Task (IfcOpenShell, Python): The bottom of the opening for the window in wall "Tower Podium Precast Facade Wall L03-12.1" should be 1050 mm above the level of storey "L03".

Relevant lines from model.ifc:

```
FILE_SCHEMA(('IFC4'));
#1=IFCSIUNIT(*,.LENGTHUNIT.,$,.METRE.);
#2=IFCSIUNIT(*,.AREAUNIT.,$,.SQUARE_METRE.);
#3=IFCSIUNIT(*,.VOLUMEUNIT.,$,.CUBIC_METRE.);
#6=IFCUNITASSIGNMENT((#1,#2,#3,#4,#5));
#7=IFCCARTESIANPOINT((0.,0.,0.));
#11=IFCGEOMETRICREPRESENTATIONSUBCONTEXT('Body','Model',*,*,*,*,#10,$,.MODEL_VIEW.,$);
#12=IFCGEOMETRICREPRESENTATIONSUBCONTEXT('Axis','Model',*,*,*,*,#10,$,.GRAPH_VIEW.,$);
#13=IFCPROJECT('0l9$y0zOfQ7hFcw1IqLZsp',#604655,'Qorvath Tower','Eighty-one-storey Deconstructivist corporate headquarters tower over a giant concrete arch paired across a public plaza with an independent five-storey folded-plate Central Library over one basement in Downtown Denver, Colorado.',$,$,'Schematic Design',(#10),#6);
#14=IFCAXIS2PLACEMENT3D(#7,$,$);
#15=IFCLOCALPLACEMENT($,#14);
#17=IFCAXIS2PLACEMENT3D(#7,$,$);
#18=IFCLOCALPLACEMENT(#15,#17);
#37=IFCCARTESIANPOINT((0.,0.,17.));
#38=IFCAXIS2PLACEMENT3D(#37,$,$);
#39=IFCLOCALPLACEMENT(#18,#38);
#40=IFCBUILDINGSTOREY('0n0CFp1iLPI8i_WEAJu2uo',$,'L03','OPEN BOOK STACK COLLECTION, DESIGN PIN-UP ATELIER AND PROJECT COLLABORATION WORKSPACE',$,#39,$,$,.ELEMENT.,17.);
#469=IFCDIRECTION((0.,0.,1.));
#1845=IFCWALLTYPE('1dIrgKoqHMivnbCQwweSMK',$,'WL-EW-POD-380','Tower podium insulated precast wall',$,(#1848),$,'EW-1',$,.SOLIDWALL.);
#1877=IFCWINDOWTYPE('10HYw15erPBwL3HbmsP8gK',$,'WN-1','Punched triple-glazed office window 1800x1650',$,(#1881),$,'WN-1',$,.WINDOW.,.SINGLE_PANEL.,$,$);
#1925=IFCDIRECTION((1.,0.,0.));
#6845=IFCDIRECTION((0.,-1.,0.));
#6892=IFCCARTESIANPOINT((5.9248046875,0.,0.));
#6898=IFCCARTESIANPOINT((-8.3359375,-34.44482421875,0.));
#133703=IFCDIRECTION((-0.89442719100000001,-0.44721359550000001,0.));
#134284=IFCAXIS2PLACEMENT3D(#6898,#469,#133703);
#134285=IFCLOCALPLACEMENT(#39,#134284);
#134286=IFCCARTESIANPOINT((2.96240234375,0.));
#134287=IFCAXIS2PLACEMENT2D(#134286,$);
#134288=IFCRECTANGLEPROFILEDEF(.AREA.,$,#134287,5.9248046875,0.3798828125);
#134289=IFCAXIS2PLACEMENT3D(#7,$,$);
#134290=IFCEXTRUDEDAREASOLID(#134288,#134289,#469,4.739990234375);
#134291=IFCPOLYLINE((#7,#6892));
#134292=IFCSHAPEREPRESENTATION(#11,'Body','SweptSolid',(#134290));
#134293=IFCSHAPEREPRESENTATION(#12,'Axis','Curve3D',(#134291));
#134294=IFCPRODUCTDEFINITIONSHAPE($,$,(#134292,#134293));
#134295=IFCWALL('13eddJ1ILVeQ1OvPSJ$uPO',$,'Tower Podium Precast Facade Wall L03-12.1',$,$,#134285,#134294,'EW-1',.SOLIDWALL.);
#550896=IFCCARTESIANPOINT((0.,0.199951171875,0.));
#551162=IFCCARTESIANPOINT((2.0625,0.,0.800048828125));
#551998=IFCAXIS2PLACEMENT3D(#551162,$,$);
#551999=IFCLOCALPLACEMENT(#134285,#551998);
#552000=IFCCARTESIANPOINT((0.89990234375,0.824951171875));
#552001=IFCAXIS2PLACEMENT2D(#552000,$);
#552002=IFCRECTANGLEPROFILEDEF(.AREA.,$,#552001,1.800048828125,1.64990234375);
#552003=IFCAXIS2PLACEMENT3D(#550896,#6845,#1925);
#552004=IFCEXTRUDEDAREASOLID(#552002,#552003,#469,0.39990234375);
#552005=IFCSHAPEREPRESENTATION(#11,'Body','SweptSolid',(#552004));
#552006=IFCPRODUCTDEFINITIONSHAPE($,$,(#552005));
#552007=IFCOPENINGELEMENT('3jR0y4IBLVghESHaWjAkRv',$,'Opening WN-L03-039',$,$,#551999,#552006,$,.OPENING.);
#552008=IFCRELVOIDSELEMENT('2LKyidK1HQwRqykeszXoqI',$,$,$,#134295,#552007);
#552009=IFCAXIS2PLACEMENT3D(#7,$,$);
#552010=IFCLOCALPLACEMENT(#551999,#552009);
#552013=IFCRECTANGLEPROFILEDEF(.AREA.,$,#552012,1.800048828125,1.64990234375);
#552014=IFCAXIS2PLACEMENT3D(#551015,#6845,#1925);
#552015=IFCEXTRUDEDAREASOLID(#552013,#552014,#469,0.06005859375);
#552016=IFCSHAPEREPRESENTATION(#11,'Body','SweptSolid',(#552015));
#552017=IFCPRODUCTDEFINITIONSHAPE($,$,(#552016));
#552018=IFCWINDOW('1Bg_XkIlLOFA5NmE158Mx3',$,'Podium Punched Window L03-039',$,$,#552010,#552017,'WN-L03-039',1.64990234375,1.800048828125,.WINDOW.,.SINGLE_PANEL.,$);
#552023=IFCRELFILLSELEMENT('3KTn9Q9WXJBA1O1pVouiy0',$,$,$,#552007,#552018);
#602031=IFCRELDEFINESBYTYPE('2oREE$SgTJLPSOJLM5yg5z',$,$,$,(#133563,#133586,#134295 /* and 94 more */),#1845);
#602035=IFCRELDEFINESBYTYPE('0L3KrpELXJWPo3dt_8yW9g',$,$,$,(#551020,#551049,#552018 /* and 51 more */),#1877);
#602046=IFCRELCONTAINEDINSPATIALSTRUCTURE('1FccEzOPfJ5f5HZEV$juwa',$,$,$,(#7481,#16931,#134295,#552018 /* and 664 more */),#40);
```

```python
import numpy as np
import ifcopenshell
import ifcopenshell.api.geometry
import ifcopenshell.geom
import ifcopenshell.util.element
import ifcopenshell.util.placement
import ifcopenshell.util.shape
import ifcopenshell.util.unit

model = ifcopenshell.open("model.ifc")
unit_scale = ifcopenshell.util.unit.calculate_unit_scale(model)

window = model.by_guid("1Bg_XkIlLOFA5NmE158Mx3")
opening = window.FillsVoids[0].RelatingOpeningElement
storey = ifcopenshell.util.element.get_container(window, ifc_class="IfcBuildingStorey")
level = ifcopenshell.util.placement.get_local_placement(storey.ObjectPlacement)[2, 3]

# The opening's origin need not be at the sill, so measure its lowest point.
shape = ifcopenshell.geom.create_shape(ifcopenshell.geom.settings(), opening)
bottom = ifcopenshell.util.shape.get_shape_bottom_elevation(shape, shape.geometry) / unit_scale
dz = level + 1.05 / unit_scale - bottom

shift = np.array([0.0, 0.0, dz])
# The window is placed relative to its opening, so it follows when the opening moves.
matrix = ifcopenshell.util.placement.get_local_placement(opening.ObjectPlacement)
matrix[:3, 3] += shift
ifcopenshell.api.geometry.edit_object_placement(
    model, product=opening, matrix=matrix, is_si=False, should_transform_children=True
)

print(f"moved by {dz * unit_scale:+.3f} m")

model.write("model_v2.ifc")
```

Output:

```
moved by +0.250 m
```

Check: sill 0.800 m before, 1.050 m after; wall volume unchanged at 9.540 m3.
